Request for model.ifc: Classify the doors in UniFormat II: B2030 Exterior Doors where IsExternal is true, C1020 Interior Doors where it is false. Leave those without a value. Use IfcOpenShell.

First a look at what the model holds.

```python
import ifcopenshell
import ifcopenshell.util.element

model = ifcopenshell.open("model.ifc")
print(model.schema)
print("classifications:", [c.Name for c in model.by_type("IfcClassification")])
values = [ifcopenshell.util.element.get_pset(e, "Pset_DoorCommon", "IsExternal") for e in model.by_type("IfcDoor")]
for value in (True, False, None):
    print("IsExternal", value, values.count(value))
```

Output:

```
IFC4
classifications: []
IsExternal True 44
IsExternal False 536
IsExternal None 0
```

```python
import ifcopenshell
import ifcopenshell.api.classification
import ifcopenshell.util.element

model = ifcopenshell.open("model.ifc")

system = ifcopenshell.api.classification.add_classification(model, classification="UniFormat II")

doors = model.by_type("IfcDoor")
external = {e: ifcopenshell.util.element.get_pset(e, "Pset_DoorCommon", "IsExternal") for e in doors}
for flag, code, name in ((True, "B2030", "Exterior Doors"), (False, "C1020", "Interior Doors")):
    products = [e for e in doors if external[e] is flag]
    ifcopenshell.api.classification.add_reference(
        model, products=products, classification=system, identification=code, name=name
    )
    print(code, len(products))

model.write("model-out.ifc")
```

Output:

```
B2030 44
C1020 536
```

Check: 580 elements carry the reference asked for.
